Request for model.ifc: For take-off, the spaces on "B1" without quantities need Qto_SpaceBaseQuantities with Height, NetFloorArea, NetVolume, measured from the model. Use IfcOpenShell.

First a look at what the model holds.

```python
import ifcopenshell
import ifcopenshell.util.element
import ifcopenshell.util.unit

model = ifcopenshell.open("model.ifc")
print(model.schema)
for unit_type in ("LENGTHUNIT", "AREAUNIT", "VOLUMEUNIT"):
    print(unit_type, ifcopenshell.util.unit.calculate_unit_scale(model, unit_type))
storey = next(s for s in model.by_type("IfcBuildingStorey") if s.Name == "B1")
spaces = [e for e in ifcopenshell.util.element.get_decomposition(storey) if e.is_a("IfcSpace")]
for e in sorted(spaces, key=lambda e: e.id()):
    print(e.id(), e.is_a(), e.Name, list(ifcopenshell.util.element.get_psets(e, qtos_only=True)), sep=" | ")
```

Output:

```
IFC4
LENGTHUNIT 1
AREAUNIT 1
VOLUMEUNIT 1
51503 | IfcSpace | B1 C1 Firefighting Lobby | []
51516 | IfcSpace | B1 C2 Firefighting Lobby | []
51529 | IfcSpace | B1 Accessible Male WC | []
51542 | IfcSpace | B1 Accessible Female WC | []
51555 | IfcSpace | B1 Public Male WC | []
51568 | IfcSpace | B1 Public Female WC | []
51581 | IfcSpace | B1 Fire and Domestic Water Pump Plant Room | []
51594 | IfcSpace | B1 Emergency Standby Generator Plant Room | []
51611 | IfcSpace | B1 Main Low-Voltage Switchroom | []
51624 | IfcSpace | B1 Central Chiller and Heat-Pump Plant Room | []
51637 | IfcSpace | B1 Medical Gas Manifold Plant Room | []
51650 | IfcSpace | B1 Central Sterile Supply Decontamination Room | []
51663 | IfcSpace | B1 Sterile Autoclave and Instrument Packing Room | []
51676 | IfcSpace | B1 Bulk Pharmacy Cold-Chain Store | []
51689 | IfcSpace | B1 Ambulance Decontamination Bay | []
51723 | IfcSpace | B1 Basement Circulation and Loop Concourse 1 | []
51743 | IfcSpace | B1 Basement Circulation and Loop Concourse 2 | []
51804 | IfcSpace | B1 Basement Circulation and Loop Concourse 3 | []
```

```python
import ifcopenshell
import ifcopenshell.api.pset
import ifcopenshell.geom
import ifcopenshell.util.element
import ifcopenshell.util.shape
import ifcopenshell.util.unit

model = ifcopenshell.open("model.ifc")
unit_scale = ifcopenshell.util.unit.calculate_unit_scale(model)
area_scale = ifcopenshell.util.unit.calculate_unit_scale(model, "AREAUNIT")
volume_scale = ifcopenshell.util.unit.calculate_unit_scale(model, "VOLUMEUNIT")
settings = ifcopenshell.geom.settings()

storey = next(s for s in model.by_type("IfcBuildingStorey") if s.Name == "B1")
spaces = [e for e in ifcopenshell.util.element.get_decomposition(storey) if e.is_a("IfcSpace")]

for e in sorted(spaces, key=lambda e: e.id()):
    if ifcopenshell.util.element.get_psets(e, qtos_only=True, should_inherit=False):
        continue
    # Geometry comes back in metres, in the element's own axes.
    shape = ifcopenshell.geom.create_shape(settings, e)
    values = {
        "Height": ifcopenshell.util.shape.get_z(shape.geometry) / unit_scale,
        "NetFloorArea": ifcopenshell.util.shape.get_footprint_area(shape.geometry) / area_scale,
        "NetVolume": ifcopenshell.util.shape.get_volume(shape.geometry) / volume_scale,
    }
    qto = ifcopenshell.api.pset.add_qto(model, product=e, name="Qto_SpaceBaseQuantities")
    ifcopenshell.api.pset.edit_qto(model, qto=qto, properties=values)
    print(e.id(), {k: round(v, 3) for k, v in values.items()})

model.write("model-out.ifc")
```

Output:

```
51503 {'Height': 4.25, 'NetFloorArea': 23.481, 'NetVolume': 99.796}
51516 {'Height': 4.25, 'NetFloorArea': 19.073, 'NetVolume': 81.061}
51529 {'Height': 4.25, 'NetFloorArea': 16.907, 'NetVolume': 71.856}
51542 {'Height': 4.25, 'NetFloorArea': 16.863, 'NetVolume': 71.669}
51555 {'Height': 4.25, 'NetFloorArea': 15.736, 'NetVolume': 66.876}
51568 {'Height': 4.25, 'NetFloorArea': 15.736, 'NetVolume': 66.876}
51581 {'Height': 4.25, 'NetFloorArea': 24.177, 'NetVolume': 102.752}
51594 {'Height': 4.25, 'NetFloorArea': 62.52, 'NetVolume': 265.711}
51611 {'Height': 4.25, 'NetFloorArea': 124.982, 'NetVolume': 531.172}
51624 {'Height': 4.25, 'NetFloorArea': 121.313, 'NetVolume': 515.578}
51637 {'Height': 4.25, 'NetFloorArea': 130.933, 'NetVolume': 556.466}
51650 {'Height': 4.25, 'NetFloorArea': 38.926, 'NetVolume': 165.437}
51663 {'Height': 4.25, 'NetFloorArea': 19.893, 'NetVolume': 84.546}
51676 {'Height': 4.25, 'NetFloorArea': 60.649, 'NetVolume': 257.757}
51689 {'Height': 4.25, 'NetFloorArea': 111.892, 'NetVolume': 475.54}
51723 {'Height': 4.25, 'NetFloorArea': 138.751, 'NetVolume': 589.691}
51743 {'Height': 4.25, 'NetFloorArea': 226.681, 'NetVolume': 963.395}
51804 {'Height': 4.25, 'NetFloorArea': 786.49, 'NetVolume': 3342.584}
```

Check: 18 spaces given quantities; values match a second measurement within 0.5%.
